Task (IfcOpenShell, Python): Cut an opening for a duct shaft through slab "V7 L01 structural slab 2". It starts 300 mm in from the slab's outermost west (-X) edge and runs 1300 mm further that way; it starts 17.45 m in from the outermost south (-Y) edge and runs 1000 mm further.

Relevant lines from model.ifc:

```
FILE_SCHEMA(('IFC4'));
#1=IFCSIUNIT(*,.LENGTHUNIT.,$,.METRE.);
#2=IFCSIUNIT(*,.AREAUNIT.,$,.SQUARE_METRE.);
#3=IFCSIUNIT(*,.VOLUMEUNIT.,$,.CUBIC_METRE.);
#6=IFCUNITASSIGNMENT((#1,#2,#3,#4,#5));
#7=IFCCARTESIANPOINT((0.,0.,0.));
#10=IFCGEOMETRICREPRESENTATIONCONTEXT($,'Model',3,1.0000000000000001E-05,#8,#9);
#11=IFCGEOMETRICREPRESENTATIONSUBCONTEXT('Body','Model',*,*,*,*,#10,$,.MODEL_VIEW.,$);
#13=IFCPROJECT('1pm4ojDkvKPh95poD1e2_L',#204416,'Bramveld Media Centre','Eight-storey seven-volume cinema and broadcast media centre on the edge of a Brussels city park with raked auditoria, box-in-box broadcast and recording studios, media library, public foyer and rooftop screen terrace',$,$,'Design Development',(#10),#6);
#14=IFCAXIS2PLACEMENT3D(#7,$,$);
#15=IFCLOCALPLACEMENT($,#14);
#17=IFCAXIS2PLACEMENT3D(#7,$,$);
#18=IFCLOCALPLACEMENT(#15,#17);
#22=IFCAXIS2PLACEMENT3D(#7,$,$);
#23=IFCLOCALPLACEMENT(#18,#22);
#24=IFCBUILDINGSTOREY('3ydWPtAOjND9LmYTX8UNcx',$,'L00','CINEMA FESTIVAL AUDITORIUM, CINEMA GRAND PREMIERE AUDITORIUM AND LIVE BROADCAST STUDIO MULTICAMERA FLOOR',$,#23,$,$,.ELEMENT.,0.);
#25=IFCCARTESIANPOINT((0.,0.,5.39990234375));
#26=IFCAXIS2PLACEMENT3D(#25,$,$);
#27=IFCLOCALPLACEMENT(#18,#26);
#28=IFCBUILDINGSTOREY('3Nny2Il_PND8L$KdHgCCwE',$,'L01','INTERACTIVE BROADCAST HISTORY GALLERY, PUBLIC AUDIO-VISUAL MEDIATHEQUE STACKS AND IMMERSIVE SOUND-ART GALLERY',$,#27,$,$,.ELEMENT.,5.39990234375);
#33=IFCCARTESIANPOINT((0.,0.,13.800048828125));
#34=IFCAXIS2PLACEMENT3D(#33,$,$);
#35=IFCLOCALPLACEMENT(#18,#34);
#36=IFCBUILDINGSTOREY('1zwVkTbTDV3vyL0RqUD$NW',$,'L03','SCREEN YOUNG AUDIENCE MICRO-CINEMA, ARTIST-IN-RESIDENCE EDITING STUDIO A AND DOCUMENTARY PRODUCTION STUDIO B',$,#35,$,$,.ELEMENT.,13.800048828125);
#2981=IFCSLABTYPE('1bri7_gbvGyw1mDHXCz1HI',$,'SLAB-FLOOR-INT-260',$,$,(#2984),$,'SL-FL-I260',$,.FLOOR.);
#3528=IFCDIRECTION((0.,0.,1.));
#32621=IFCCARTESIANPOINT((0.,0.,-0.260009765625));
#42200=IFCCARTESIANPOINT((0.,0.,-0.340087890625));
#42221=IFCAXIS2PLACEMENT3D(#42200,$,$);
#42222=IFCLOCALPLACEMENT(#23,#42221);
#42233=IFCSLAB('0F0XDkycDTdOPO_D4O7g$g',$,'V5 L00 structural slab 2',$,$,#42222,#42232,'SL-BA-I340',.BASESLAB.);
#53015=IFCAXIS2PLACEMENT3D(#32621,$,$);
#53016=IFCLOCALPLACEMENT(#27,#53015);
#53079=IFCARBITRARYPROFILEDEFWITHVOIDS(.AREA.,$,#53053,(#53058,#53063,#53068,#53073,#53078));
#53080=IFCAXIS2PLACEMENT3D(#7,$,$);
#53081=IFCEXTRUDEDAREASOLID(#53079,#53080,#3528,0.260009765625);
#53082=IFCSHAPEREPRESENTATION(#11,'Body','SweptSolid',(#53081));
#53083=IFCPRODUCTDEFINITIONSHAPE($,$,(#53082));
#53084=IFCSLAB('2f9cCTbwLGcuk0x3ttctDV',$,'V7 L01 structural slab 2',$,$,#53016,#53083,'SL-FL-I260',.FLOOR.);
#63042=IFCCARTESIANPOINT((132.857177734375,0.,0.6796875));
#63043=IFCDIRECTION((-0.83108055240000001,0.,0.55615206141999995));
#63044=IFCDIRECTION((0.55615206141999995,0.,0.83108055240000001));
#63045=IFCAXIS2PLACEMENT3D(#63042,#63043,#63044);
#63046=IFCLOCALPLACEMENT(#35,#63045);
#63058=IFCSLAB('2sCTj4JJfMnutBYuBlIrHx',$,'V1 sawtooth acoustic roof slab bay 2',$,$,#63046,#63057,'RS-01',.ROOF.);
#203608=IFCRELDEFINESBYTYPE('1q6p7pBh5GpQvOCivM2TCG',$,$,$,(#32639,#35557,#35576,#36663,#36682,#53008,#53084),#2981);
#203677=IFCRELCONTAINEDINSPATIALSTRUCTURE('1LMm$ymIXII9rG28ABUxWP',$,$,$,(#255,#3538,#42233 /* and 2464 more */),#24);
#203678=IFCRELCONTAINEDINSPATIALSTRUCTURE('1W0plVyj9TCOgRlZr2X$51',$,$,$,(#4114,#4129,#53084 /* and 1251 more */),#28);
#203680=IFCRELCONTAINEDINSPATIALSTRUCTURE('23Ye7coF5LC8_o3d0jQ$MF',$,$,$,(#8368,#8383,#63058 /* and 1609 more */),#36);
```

```python
import numpy as np
import ifcopenshell
import ifcopenshell.api.feature
import ifcopenshell.api.geometry
import ifcopenshell.api.root
import ifcopenshell.geom
import ifcopenshell.util.placement
import ifcopenshell.util.representation
import ifcopenshell.util.shape
import ifcopenshell.util.unit

model = ifcopenshell.open("model.ifc")
unit_scale = ifcopenshell.util.unit.calculate_unit_scale(model)
settings = ifcopenshell.geom.settings()


def volume(element):
    """Net volume in cubic metres, openings subtracted."""
    shape = ifcopenshell.geom.create_shape(settings, element)
    return ifcopenshell.util.shape.get_volume(shape.geometry)


slab = model.by_guid("2f9cCTbwLGcuk0x3ttctDV")
before = volume(slab)

# Extent in the slab's own axes, in metres. The edges named are its -X and -Y sides.
slab_shape = ifcopenshell.geom.create_shape(settings, slab)
vertices = ifcopenshell.util.shape.get_vertices(slab_shape.geometry)
x_min, y_min, bottom = vertices.min(axis=0)
top = vertices[:, 2].max()

opening = ifcopenshell.api.root.create_entity(model, ifc_class="IfcOpeningElement", name="Duct shaft opening", predefined_type="OPENING")
context = ifcopenshell.util.representation.get_context(model, "Model", "Body", "MODEL_VIEW")
width, depth = 1.3, 1
outline = [(0.0, 0.0), (width, 0.0), (width, depth), (0.0, depth), (0.0, 0.0)]
# Overshoot both faces by 50 mm so the cut is clean.
shape = ifcopenshell.api.geometry.add_slab_representation(
    model, context=context, depth=top - bottom + 0.1, polyline=outline
)
ifcopenshell.api.geometry.assign_representation(model, product=opening, representation=shape)

matrix = ifcopenshell.util.placement.get_local_placement(slab.ObjectPlacement)
matrix[:, 3] = matrix @ np.append(np.array([x_min + 0.3, y_min + 17.45, bottom - 0.05]) / unit_scale, 1.0)
ifcopenshell.api.geometry.edit_object_placement(model, product=opening, matrix=matrix, is_si=False)
ifcopenshell.api.feature.add_feature(model, feature=opening, element=slab)

after = volume(slab)

print(f"slab volume {before:.3f} -> {after:.3f} m3")

model.write("model_updated.ifc")
```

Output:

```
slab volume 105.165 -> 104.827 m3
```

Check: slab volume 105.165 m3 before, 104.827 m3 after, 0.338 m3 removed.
